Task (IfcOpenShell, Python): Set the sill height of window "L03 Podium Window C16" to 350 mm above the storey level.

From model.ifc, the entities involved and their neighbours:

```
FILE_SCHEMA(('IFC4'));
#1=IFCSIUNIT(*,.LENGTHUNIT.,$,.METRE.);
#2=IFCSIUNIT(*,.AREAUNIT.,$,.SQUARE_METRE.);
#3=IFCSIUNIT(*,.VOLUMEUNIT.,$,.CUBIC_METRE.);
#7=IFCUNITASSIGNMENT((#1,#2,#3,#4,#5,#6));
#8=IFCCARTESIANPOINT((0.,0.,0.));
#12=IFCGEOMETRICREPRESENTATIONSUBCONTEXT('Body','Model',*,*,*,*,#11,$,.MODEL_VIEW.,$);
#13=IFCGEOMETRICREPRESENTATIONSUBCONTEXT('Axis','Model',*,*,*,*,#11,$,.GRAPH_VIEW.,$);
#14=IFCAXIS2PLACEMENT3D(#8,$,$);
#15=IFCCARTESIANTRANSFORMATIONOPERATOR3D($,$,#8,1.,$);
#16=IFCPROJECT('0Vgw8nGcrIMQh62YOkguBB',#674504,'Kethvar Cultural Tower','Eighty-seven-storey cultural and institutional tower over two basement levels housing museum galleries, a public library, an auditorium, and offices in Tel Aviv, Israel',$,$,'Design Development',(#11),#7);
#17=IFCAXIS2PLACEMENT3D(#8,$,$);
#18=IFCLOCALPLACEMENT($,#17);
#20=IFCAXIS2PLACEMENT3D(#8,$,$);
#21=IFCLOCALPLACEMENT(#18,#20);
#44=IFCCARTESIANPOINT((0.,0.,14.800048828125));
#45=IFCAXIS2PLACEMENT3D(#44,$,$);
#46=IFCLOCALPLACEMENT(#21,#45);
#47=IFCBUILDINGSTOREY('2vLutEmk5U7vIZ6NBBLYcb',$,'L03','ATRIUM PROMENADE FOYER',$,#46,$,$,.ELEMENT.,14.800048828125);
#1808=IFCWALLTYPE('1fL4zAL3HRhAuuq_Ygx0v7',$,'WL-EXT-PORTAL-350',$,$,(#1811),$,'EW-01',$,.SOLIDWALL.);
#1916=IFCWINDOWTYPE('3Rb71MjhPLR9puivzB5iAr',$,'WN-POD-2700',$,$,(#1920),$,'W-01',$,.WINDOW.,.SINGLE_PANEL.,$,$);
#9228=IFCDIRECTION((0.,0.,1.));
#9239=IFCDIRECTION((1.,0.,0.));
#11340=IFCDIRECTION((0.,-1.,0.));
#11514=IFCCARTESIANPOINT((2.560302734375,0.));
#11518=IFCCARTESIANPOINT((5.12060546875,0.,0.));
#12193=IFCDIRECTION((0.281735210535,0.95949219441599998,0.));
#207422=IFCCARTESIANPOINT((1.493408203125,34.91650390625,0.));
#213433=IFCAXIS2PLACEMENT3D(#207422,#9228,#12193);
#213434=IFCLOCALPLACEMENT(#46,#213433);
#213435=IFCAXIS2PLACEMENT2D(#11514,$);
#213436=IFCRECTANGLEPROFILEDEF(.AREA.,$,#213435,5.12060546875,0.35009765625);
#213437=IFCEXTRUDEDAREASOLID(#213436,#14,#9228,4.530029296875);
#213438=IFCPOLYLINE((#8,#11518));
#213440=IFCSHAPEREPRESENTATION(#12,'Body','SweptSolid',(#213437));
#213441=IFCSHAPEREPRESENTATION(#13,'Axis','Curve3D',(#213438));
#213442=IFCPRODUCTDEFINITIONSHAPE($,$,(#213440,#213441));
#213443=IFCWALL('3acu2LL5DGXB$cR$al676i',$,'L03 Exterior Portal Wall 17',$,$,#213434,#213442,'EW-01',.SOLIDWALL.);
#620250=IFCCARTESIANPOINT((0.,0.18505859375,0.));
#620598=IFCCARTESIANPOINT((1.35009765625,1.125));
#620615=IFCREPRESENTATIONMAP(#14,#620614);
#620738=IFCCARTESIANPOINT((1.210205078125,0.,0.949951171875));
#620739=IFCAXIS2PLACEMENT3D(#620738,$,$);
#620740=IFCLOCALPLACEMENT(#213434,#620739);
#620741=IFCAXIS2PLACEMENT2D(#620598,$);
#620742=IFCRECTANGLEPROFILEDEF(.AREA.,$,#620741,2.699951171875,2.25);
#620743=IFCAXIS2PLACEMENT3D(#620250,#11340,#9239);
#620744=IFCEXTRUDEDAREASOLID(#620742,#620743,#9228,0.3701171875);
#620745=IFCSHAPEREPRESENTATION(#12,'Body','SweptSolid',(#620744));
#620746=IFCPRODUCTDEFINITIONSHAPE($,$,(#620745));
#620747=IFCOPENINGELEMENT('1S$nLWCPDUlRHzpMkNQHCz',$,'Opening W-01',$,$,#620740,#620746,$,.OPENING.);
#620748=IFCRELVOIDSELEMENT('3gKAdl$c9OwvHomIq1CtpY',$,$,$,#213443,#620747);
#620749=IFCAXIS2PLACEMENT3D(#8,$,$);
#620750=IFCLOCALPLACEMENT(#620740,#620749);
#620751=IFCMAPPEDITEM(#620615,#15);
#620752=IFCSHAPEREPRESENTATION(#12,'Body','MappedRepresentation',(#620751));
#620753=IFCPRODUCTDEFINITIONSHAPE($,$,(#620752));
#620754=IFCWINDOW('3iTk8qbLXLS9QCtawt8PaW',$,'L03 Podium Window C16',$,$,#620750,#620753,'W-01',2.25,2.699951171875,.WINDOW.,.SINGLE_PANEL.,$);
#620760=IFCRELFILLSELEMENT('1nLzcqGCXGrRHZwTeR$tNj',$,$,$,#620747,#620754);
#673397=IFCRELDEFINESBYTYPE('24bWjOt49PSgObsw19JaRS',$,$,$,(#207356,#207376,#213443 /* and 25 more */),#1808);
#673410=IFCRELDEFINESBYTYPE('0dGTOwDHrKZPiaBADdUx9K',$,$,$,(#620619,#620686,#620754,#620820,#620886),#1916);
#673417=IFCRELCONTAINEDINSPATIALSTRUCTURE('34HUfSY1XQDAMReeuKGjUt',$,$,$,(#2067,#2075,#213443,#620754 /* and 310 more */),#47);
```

```python
import numpy as np
import ifcopenshell
import ifcopenshell.api.geometry
import ifcopenshell.geom
import ifcopenshell.util.element
import ifcopenshell.util.placement
import ifcopenshell.util.shape
import ifcopenshell.util.unit

model = ifcopenshell.open("model.ifc")
unit_scale = ifcopenshell.util.unit.calculate_unit_scale(model)

window = model.by_guid("3iTk8qbLXLS9QCtawt8PaW")
opening = window.FillsVoids[0].RelatingOpeningElement
storey = ifcopenshell.util.element.get_container(window, ifc_class="IfcBuildingStorey")
level = ifcopenshell.util.placement.get_local_placement(storey.ObjectPlacement)[2, 3]

# The opening's origin need not be at the sill, so measure its lowest point.
shape = ifcopenshell.geom.create_shape(ifcopenshell.geom.settings(), opening)
bottom = ifcopenshell.util.shape.get_shape_bottom_elevation(shape, shape.geometry) / unit_scale
dz = level + 0.35 - bottom

shift = np.array([0.0, 0.0, dz])
# The window is placed relative to its opening, so it follows when the opening moves.
matrix = ifcopenshell.util.placement.get_local_placement(opening.ObjectPlacement)
matrix[:3, 3] += shift
ifcopenshell.api.geometry.edit_object_placement(
    model, product=opening, matrix=matrix, is_si=False, should_transform_children=True
)

print(f"moved by {dz * unit_scale:+.3f} m")

model.write("model-out.ifc")
```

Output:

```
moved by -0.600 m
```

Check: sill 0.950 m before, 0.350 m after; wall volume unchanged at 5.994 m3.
